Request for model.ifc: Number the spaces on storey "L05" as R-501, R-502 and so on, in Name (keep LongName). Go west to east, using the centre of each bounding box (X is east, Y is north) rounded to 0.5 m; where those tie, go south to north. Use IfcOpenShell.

First a look at what the model holds.

```python
import ifcopenshell
import ifcopenshell.util.element
import ifcopenshell.util.placement

model = ifcopenshell.open("model.ifc")
print(model.schema)
storey = next(s for s in model.by_type("IfcBuildingStorey") if s.Name == "L05")
spaces = [e for e in ifcopenshell.util.element.get_decomposition(storey) if e.is_a("IfcSpace")]
for e in sorted(spaces, key=lambda e: e.id()):
    origin = ifcopenshell.util.placement.get_local_placement(e.ObjectPlacement)[:3, 3]
    print(e.id(), e.Name, e.LongName, origin.round(2) + 0.0, sep=" | ")
```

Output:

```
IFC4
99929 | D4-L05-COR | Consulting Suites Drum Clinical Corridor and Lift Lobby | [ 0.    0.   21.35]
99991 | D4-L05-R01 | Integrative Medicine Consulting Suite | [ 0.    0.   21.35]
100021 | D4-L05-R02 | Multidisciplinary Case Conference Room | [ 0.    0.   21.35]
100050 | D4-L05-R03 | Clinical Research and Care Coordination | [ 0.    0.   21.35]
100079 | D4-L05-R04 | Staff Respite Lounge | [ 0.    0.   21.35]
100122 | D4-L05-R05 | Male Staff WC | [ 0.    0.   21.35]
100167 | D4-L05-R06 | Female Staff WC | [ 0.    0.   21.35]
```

```python
import ifcopenshell
import ifcopenshell.geom
import ifcopenshell.util.element
import ifcopenshell.util.shape

model = ifcopenshell.open("model.ifc")
settings = ifcopenshell.geom.settings()
settings.set("use-world-coords", True)


def centre(element):
    shape = ifcopenshell.geom.create_shape(settings, element)
    return ifcopenshell.util.shape.get_bbox_centroid(shape.geometry)


storey = next(s for s in model.by_type("IfcBuildingStorey") if s.Name == "L05")
spaces = [e for e in ifcopenshell.util.element.get_decomposition(storey) if e.is_a("IfcSpace")]

# Insertion points can sit at a corner or the storey origin, so sort by the geometry (in metres).
centres = {e: centre(e) for e in spaces}
spaces.sort(key=lambda e: (round(centres[e][0] / 0.5), centres[e][1]))

for i, e in enumerate(spaces, start=1):
    number = f"R-5{i:02d}"
    e.Name = number
    print(e.id(), number)

model.write("model_updated.ifc")
```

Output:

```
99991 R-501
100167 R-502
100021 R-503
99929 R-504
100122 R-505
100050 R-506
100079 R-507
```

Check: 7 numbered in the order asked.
